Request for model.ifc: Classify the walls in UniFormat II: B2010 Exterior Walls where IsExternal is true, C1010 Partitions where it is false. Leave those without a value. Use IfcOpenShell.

First a look at what the model holds.

```python
import ifcopenshell
import ifcopenshell.util.element

model = ifcopenshell.open("model.ifc")
print(model.schema)
print("classifications:", [c.Name for c in model.by_type("IfcClassification")])
values = [ifcopenshell.util.element.get_pset(e, "Pset_WallCommon", "IsExternal") for e in model.by_type("IfcWall")]
for value in (True, False, None):
    print("IsExternal", value, values.count(value))
```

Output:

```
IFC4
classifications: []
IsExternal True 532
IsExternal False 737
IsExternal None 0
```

```python
import ifcopenshell
import ifcopenshell.api.classification
import ifcopenshell.util.element

model = ifcopenshell.open("model.ifc")

system = ifcopenshell.api.classification.add_classification(model, classification="UniFormat II")

walls = model.by_type("IfcWall")
external = {e: ifcopenshell.util.element.get_pset(e, "Pset_WallCommon", "IsExternal") for e in walls}
for flag, code, name in ((True, "B2010", "Exterior Walls"), (False, "C1010", "Partitions")):
    products = [e for e in walls if external[e] is flag]
    ifcopenshell.api.classification.add_reference(
        model, products=products, classification=system, identification=code, name=name
    )
    print(code, len(products))

model.write("model_updated.ifc")
```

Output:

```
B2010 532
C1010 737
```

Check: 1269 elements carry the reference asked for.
